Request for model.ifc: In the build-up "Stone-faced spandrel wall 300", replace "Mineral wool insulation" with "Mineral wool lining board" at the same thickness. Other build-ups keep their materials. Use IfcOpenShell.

First a look at what the model holds.

```python
import ifcopenshell
import ifcopenshell.util.element

model = ifcopenshell.open("model.ifc")
print(model.schema)
for layer_set in model.by_type("IfcMaterialLayerSet"):
    if layer_set.LayerSetName == "Stone-faced spandrel wall 300":
        for layer in layer_set.MaterialLayers:
            print(layer.id(), layer.Material and layer.Material.Name, layer.LayerThickness, sep=" | ")
        print(len(ifcopenshell.util.element.get_elements_by_material(model, layer_set)), "elements and types use it")
print(sorted(m.Name for m in model.by_type("IfcMaterial") if m.Name)[:60])
```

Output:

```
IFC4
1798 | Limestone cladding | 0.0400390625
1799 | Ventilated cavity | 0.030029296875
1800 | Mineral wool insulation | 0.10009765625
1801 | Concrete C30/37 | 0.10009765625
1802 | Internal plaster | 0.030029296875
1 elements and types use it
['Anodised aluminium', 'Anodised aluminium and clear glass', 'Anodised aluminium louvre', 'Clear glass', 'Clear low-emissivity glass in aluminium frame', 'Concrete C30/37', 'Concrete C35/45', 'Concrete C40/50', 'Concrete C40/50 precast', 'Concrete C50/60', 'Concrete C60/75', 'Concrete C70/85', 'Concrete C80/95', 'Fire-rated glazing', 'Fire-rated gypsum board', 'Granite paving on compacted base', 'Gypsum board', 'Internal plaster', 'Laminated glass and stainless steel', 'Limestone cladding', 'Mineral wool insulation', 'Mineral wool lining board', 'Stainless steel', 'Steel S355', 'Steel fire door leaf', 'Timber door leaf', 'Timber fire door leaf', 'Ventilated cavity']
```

```python
import ifcopenshell
import ifcopenshell.api.material

model = ifcopenshell.open("model.ifc")

layer_set = next(s for s in model.by_type("IfcMaterialLayerSet") if s.LayerSetName == "Stone-faced spandrel wall 300")
layer = next(l for l in layer_set.MaterialLayers if l.Material and l.Material.Name == "Mineral wool insulation")
material = next(m for m in model.by_type("IfcMaterial") if m.Name == "Mineral wool lining board")

# Point this one layer at the other material; renaming the old one would change it everywhere.
ifcopenshell.api.material.edit_layer(model, layer=layer, attributes={}, material=material)

print([l.Material.Name if l.Material else None for l in layer_set.MaterialLayers])

model.write("model_edited.ifc")
```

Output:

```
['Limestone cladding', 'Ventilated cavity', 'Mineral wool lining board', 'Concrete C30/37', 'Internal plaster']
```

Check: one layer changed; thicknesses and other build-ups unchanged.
